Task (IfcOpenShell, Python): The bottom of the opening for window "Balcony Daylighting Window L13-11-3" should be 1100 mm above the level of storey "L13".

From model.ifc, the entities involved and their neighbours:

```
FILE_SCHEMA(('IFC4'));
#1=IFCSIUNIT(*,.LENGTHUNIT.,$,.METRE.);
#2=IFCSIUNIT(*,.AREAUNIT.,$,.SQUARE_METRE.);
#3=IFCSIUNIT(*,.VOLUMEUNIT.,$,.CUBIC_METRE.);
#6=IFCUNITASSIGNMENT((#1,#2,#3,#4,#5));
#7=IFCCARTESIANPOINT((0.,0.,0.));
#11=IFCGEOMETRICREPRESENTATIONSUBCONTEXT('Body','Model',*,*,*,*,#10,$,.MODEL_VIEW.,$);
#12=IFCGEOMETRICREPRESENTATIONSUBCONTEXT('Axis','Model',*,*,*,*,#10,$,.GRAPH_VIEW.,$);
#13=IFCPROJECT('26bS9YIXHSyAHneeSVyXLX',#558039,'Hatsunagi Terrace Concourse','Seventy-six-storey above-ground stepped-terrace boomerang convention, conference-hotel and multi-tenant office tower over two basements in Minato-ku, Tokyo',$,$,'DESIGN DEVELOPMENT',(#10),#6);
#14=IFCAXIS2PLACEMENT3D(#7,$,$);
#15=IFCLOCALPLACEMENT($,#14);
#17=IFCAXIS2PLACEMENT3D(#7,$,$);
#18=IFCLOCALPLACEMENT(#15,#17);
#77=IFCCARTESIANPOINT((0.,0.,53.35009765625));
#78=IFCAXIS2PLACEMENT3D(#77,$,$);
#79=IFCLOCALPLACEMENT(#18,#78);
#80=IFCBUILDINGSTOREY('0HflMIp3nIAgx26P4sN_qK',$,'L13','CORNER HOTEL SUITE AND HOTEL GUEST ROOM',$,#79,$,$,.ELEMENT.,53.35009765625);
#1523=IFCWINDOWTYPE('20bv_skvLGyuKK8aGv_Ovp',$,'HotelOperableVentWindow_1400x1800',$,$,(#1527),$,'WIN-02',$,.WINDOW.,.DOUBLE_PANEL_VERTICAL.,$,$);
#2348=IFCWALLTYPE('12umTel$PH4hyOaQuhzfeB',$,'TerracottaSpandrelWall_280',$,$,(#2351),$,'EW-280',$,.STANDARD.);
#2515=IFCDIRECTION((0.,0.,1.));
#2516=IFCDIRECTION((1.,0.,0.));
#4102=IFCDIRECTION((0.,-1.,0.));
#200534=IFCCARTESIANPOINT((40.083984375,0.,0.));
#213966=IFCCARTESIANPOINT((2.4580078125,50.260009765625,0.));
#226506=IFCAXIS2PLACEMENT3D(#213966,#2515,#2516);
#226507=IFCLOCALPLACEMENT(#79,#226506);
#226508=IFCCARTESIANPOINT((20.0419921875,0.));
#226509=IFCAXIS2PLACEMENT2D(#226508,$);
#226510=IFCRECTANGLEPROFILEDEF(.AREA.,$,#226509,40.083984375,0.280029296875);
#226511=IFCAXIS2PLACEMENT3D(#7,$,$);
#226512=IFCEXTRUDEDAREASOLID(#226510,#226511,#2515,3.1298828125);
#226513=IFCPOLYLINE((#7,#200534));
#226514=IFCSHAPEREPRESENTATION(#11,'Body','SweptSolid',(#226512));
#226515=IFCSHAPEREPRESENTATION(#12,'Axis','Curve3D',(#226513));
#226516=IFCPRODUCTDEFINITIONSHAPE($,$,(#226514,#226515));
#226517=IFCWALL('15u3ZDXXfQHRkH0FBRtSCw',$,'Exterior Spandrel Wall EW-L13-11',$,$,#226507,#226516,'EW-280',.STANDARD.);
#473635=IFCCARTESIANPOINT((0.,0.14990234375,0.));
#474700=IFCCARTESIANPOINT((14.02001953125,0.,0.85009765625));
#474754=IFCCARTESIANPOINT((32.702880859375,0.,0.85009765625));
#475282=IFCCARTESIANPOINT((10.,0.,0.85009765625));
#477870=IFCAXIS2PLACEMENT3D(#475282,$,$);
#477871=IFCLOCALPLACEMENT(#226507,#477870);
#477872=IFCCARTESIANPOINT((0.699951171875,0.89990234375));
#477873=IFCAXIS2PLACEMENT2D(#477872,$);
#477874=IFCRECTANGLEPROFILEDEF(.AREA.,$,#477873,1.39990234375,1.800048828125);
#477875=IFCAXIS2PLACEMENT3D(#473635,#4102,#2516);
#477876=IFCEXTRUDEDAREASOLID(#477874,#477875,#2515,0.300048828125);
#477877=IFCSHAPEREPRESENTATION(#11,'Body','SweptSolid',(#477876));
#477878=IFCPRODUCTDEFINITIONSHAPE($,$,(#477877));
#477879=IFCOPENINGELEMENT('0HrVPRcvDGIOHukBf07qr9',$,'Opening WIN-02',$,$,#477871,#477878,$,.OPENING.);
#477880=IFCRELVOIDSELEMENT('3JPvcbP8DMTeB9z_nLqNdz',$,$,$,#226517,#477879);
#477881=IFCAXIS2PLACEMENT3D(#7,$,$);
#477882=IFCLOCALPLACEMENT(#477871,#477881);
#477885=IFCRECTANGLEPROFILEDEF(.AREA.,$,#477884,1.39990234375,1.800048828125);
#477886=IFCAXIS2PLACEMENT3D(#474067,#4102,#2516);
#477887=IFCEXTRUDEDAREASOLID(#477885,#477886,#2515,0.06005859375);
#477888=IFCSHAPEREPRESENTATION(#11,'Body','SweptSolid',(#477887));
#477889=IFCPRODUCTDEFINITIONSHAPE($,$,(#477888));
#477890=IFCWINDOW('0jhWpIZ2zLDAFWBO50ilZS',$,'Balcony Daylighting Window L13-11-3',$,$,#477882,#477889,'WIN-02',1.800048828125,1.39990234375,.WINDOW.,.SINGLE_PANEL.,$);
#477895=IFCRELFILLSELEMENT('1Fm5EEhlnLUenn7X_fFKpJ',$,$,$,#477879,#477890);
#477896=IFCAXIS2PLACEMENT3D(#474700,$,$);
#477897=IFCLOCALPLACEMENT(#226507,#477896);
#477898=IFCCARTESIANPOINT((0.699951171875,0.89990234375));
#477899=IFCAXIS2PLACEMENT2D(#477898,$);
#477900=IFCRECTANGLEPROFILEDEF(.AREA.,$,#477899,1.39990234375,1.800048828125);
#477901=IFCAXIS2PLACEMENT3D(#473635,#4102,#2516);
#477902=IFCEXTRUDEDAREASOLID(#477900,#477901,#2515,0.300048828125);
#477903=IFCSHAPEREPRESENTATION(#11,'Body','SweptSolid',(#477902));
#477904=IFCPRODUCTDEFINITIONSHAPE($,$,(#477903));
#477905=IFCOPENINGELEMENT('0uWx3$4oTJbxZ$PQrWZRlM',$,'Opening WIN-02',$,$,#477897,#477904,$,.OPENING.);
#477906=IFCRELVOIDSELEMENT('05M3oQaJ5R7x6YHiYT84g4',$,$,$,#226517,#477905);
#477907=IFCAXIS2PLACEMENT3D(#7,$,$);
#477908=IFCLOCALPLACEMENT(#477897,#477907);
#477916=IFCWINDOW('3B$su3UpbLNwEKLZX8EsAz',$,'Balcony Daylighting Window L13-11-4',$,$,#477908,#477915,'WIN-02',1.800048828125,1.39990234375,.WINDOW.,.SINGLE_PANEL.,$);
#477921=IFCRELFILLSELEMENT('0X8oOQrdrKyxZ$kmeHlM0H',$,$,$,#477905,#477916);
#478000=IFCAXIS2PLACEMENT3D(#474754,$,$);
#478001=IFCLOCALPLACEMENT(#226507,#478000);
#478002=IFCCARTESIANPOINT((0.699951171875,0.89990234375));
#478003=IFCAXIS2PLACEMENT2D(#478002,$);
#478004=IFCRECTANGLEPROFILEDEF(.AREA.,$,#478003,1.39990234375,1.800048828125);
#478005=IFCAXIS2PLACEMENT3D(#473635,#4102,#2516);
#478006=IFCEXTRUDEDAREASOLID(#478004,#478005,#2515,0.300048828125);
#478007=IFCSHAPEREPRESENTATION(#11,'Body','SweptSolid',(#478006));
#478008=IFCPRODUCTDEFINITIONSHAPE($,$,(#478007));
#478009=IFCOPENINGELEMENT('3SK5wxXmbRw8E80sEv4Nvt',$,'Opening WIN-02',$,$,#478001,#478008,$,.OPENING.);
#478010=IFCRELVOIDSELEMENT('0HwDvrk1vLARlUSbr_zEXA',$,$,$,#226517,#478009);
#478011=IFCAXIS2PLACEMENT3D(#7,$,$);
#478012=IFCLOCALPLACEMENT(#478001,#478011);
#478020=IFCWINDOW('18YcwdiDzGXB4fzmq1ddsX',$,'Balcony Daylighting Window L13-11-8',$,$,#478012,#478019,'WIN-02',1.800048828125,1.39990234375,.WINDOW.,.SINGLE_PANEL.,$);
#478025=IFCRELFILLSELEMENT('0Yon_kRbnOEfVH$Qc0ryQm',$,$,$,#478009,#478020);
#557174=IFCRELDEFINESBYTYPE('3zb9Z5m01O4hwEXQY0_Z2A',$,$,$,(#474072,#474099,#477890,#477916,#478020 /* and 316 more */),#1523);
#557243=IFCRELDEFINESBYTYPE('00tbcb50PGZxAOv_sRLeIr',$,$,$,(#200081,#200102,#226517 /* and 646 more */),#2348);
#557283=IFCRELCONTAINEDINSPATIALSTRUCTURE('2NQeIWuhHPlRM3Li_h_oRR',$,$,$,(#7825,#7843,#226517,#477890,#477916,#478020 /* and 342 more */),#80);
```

```python
import numpy as np
import ifcopenshell
import ifcopenshell.api.geometry
import ifcopenshell.geom
import ifcopenshell.util.element
import ifcopenshell.util.placement
import ifcopenshell.util.shape
import ifcopenshell.util.unit

model = ifcopenshell.open("model.ifc")
unit_scale = ifcopenshell.util.unit.calculate_unit_scale(model)

window = model.by_guid("0jhWpIZ2zLDAFWBO50ilZS")
opening = window.FillsVoids[0].RelatingOpeningElement
storey = ifcopenshell.util.element.get_container(window, ifc_class="IfcBuildingStorey")
level = ifcopenshell.util.placement.get_local_placement(storey.ObjectPlacement)[2, 3]

# The opening's origin need not be at the sill, so measure its lowest point.
shape = ifcopenshell.geom.create_shape(ifcopenshell.geom.settings(), opening)
bottom = ifcopenshell.util.shape.get_shape_bottom_elevation(shape, shape.geometry) / unit_scale
dz = level + 1.1 - bottom

shift = np.array([0.0, 0.0, dz])
# The window is placed relative to its opening, so it follows when the opening moves.
matrix = ifcopenshell.util.placement.get_local_placement(opening.ObjectPlacement)
matrix[:3, 3] += shift
ifcopenshell.api.geometry.edit_object_placement(
    model, product=opening, matrix=matrix, is_si=False, should_transform_children=True
)

print(f"moved by {dz * unit_scale:+.3f} m")

model.write("model_updated.ifc")
```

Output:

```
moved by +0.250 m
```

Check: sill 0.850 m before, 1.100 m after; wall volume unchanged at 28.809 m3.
